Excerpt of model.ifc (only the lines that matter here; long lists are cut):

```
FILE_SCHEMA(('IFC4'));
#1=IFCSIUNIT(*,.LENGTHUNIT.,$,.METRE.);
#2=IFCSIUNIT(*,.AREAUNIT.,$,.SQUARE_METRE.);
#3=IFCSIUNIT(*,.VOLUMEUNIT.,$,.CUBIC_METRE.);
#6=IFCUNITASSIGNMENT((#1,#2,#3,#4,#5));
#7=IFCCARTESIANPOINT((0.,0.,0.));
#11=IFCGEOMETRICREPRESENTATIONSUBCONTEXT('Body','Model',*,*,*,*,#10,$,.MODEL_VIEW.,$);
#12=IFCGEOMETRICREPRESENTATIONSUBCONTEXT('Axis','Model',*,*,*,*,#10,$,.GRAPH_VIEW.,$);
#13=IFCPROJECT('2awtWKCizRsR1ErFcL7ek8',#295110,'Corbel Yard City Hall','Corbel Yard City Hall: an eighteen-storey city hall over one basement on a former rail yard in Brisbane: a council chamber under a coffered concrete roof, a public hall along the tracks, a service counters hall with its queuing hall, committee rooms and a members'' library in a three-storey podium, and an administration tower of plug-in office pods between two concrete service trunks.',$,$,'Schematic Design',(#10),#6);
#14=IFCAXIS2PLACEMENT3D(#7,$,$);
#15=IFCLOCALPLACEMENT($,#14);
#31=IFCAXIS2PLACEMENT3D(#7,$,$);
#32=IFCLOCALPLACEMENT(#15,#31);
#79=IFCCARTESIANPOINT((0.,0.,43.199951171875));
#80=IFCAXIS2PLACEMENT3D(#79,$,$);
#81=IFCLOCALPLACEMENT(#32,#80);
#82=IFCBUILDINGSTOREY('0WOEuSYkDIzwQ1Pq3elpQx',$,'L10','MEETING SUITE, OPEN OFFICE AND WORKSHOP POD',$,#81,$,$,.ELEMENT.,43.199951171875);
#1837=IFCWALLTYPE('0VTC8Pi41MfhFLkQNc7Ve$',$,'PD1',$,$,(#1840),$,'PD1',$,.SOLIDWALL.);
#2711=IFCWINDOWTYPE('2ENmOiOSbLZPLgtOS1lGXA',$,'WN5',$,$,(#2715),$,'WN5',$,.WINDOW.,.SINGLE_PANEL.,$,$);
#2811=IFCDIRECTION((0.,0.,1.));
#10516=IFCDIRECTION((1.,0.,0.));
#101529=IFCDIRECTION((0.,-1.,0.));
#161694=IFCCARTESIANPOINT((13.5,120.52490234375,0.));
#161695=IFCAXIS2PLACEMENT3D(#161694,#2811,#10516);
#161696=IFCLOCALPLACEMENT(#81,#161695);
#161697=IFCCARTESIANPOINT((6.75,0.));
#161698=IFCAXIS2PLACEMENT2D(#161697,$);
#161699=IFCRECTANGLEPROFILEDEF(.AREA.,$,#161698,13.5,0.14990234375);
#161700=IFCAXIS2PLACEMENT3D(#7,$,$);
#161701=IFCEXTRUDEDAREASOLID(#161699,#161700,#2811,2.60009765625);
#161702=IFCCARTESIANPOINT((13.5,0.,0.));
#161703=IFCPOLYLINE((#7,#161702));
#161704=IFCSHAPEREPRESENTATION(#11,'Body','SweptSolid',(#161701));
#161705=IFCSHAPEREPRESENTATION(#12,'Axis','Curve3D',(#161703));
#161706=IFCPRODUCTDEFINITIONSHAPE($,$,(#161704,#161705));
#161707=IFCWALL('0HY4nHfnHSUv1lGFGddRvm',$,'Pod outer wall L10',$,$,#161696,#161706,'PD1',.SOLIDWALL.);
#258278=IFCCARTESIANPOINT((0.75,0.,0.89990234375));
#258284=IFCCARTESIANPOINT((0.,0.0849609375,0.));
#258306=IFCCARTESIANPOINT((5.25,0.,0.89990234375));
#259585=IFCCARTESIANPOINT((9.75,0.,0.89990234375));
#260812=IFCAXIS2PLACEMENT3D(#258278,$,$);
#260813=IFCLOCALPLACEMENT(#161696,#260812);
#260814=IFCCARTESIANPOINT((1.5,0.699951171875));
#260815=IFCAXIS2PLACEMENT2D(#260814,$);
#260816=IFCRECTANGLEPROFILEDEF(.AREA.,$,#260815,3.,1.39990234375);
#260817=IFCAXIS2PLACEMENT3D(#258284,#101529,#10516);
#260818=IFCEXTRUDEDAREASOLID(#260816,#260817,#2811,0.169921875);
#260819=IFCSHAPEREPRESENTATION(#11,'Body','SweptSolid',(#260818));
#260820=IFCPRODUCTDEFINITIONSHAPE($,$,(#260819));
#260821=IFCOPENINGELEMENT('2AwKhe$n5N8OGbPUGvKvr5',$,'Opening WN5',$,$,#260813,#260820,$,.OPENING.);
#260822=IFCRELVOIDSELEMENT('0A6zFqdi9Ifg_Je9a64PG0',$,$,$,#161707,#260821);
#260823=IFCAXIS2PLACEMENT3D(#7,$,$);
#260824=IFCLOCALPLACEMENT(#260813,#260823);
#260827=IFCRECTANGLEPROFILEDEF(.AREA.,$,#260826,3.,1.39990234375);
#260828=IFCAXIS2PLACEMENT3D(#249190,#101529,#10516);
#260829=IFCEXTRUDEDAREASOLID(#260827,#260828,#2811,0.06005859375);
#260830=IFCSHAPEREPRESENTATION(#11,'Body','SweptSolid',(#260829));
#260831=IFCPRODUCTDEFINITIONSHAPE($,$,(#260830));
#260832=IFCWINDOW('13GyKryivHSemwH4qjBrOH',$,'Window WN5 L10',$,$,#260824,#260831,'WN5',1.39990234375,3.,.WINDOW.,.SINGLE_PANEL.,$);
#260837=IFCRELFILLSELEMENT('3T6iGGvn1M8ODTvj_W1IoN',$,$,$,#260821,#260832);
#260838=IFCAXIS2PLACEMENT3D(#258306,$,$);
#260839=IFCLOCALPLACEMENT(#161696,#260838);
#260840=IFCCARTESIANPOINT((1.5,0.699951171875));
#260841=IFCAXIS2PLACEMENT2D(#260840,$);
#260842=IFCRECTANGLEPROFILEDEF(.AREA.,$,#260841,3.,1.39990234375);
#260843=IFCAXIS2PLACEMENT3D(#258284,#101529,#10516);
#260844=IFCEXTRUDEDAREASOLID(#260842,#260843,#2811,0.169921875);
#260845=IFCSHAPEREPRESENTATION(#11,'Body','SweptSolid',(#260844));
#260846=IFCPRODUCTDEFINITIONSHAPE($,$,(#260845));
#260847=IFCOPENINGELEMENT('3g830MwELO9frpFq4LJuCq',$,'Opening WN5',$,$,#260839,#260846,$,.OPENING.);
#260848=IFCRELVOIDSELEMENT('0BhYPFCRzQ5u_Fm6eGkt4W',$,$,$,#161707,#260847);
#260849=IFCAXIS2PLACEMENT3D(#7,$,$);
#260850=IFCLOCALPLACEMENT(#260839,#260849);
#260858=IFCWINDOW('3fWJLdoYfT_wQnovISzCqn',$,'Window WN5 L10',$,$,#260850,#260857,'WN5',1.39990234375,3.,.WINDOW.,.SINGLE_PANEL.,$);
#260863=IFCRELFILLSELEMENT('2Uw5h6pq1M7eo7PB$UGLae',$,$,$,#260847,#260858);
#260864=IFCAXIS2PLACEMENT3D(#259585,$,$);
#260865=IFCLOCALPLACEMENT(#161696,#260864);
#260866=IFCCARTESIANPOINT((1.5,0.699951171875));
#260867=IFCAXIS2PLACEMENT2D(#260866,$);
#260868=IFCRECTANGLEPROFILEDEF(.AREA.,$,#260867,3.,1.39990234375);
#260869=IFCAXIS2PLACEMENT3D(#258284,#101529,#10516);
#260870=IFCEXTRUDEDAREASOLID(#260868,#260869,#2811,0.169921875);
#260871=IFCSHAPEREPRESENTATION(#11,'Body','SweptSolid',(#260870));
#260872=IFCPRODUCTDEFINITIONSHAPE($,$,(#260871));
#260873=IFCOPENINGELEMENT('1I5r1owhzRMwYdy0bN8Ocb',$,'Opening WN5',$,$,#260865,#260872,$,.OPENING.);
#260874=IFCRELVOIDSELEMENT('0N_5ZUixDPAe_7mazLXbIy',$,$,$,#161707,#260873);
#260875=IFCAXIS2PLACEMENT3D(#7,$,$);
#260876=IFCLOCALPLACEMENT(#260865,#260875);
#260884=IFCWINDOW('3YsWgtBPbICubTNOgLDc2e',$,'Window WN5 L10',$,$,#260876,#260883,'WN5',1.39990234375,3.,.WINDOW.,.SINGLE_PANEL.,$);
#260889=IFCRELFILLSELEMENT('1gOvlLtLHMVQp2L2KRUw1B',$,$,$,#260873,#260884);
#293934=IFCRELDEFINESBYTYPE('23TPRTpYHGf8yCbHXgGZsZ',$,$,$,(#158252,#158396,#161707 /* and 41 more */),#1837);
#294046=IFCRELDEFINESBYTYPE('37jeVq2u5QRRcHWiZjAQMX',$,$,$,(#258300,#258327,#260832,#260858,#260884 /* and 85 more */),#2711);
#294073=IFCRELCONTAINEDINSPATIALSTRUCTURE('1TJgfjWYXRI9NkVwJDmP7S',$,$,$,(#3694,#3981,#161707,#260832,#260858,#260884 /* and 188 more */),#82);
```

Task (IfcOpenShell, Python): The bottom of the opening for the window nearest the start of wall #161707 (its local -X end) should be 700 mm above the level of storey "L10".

```python
import numpy as np
import ifcopenshell
import ifcopenshell.api.geometry
import ifcopenshell.geom
import ifcopenshell.util.element
import ifcopenshell.util.placement
import ifcopenshell.util.shape
import ifcopenshell.util.unit

model = ifcopenshell.open("model.ifc")
unit_scale = ifcopenshell.util.unit.calculate_unit_scale(model)

window = model.by_id(260832)
opening = window.FillsVoids[0].RelatingOpeningElement
storey = ifcopenshell.util.element.get_container(window, ifc_class="IfcBuildingStorey")
level = ifcopenshell.util.placement.get_local_placement(storey.ObjectPlacement)[2, 3]

# The opening's origin need not be at the sill, so measure its lowest point.
shape = ifcopenshell.geom.create_shape(ifcopenshell.geom.settings(), opening)
bottom = ifcopenshell.util.shape.get_shape_bottom_elevation(shape, shape.geometry) / unit_scale
dz = level + 0.7 / unit_scale - bottom

shift = np.array([0.0, 0.0, dz])
# The window is placed relative to its opening, so it follows when the opening moves.
matrix = ifcopenshell.util.placement.get_local_placement(opening.ObjectPlacement)
matrix[:3, 3] += shift
ifcopenshell.api.geometry.edit_object_placement(
    model, product=opening, matrix=matrix, is_si=False, should_transform_children=True
)

print(f"moved by {dz * unit_scale:+.3f} m")

model.write("model_updated.ifc")
```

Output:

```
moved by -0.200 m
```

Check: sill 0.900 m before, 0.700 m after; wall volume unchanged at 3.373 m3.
